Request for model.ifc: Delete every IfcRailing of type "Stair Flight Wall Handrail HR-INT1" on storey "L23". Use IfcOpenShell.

First a look at what the model holds.

```python
import ifcopenshell
import ifcopenshell.util.element

model = ifcopenshell.open("model.ifc")
print(model.schema)
storey = next(s for s in model.by_type("IfcBuildingStorey") if s.Name == "L23")
railings = [e for e in ifcopenshell.util.element.get_decomposition(storey) if e.is_a("IfcRailing")]
seen = {}
for e in railings:
    element_type = ifcopenshell.util.element.get_type(e)
    name = element_type.Name if element_type not in (None, e) else None
    seen[name] = seen.get(name, 0) + 1
for name, count in sorted(seen.items(), key=str):
    print(count, "x", name)
```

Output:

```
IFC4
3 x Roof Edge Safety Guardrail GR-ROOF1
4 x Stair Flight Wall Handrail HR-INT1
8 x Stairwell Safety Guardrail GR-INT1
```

```python
import ifcopenshell
import ifcopenshell.api.root
import ifcopenshell.util.element

model = ifcopenshell.open("model.ifc")

storey = next(s for s in model.by_type("IfcBuildingStorey") if s.Name == "L23")
railings = [e for e in ifcopenshell.util.element.get_decomposition(storey) if e.is_a("IfcRailing")]
targets = [e for e in railings if (t := ifcopenshell.util.element.get_type(e)) not in (None, e) and t.Name == "Stair Flight Wall Handrail HR-INT1"]

for e in targets:
    ifcopenshell.api.root.remove_product(model, product=e)
print(len(targets), "removed")

model.write("model_edited.ifc")
```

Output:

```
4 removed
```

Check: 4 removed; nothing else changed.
